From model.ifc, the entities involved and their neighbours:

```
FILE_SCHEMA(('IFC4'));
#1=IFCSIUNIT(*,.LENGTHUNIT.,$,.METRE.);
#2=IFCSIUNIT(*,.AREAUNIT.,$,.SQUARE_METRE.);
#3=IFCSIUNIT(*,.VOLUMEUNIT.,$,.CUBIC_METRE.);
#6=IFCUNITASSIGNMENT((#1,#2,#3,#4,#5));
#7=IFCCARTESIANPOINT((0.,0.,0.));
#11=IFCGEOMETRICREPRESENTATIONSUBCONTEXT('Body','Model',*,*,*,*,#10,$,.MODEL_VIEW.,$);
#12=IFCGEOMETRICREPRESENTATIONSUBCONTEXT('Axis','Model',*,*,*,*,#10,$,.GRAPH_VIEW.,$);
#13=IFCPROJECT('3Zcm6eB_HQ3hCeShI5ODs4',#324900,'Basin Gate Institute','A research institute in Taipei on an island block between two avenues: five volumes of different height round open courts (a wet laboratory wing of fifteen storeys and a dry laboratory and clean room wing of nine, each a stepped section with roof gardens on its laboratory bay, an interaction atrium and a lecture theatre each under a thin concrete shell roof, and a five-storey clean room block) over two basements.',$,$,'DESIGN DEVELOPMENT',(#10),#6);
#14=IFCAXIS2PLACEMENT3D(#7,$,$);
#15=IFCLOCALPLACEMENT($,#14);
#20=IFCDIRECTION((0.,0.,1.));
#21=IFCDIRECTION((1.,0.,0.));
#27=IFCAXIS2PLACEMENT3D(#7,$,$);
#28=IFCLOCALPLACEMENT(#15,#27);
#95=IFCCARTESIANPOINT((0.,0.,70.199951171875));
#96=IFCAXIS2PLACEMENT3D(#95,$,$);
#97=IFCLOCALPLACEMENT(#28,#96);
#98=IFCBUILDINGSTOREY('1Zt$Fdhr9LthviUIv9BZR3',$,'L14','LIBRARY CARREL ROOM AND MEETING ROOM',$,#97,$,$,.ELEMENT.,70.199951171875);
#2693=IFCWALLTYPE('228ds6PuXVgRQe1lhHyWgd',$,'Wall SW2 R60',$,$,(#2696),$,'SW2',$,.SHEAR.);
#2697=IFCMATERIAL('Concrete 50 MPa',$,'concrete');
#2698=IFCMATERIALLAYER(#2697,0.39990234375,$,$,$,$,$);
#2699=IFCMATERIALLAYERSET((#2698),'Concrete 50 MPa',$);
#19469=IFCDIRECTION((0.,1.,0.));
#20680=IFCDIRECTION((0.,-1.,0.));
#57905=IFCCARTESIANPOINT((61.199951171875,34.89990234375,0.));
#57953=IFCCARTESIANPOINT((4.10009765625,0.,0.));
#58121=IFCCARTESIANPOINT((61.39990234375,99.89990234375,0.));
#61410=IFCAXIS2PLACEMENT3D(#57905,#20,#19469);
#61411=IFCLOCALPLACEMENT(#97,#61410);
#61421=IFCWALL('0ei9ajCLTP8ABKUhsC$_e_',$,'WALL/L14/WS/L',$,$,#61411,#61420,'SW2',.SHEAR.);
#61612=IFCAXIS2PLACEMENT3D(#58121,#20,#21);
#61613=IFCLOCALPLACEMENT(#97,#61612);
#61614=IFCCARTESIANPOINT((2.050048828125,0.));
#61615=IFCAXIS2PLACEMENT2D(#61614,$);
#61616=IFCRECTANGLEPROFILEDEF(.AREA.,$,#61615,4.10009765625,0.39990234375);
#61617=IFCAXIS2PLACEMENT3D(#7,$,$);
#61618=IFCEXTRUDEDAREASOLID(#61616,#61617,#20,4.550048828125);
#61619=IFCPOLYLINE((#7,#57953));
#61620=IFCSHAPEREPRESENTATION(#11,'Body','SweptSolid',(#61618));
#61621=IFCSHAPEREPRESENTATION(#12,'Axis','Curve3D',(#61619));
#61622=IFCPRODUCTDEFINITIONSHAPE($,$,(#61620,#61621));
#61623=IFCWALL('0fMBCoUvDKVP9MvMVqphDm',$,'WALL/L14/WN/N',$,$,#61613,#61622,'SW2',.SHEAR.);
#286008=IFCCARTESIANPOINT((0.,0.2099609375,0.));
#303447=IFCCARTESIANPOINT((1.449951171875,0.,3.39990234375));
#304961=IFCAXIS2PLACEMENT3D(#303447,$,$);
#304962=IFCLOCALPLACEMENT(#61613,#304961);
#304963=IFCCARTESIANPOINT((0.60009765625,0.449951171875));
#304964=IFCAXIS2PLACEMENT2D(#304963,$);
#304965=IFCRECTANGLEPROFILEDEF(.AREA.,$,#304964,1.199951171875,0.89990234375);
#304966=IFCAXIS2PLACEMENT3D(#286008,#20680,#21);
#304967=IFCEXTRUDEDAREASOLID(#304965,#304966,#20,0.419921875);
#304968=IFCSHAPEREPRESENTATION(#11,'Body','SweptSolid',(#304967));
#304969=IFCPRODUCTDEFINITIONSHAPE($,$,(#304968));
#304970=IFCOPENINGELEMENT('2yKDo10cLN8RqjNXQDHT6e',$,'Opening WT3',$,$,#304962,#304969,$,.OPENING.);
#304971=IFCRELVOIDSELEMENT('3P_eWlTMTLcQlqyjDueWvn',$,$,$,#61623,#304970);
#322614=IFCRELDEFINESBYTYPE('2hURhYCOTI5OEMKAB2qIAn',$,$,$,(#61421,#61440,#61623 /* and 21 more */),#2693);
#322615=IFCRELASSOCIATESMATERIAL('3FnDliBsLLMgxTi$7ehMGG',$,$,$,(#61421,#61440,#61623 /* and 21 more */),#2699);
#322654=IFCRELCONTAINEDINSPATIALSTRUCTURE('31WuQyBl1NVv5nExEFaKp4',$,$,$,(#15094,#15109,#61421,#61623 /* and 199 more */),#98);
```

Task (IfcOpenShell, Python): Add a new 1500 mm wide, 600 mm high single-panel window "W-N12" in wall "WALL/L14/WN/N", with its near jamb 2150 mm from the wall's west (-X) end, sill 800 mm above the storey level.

```python
import numpy as np
import ifcopenshell
import ifcopenshell.api.feature
import ifcopenshell.api.geometry
import ifcopenshell.api.root
import ifcopenshell.api.spatial
import ifcopenshell.geom
import ifcopenshell.util.element
import ifcopenshell.util.placement
import ifcopenshell.util.representation
import ifcopenshell.util.shape
import ifcopenshell.util.unit

model = ifcopenshell.open("model.ifc")
unit_scale = ifcopenshell.util.unit.calculate_unit_scale(model)
settings = ifcopenshell.geom.settings()


def volume(element):
    """Net volume in cubic metres, openings subtracted."""
    shape = ifcopenshell.geom.create_shape(settings, element)
    return ifcopenshell.util.shape.get_volume(shape.geometry)


wall = model.by_guid("0fMBCoUvDKVP9MvMVqphDm")
storey = ifcopenshell.util.element.get_container(wall, ifc_class="IfcBuildingStorey")
context = ifcopenshell.util.representation.get_context(model, "Model", "Body", "MODEL_VIEW")
before = volume(wall)

width, height, from_end, sill = 1.5, 0.6, 2.15, 0.8  # metres

# The wall runs along its own X axis, and the end named is its -X end.
wall_shape = ifcopenshell.geom.create_shape(settings, wall)
x, y, z = ifcopenshell.util.shape.get_vertices(wall_shape.geometry).T
start = x.min() + from_end
face, thickness = float(y.min()), float(y.max() - y.min())
wall_matrix = ifcopenshell.util.placement.get_local_placement(wall.ObjectPlacement)
level = ifcopenshell.util.placement.get_local_placement(storey.ObjectPlacement)[2, 3]


def in_wall(x, y):
    """Placement at x, y metres in the wall's axes, at sill height."""
    matrix = wall_matrix.copy()
    matrix[:, 3] = wall_matrix @ np.array([x / unit_scale, y / unit_scale, 0.0, 1.0])
    matrix[2, 3] = level + sill / unit_scale
    return matrix


# Opening: a box that overshoots both wall faces by 50 mm.
opening = ifcopenshell.api.root.create_entity(model, ifc_class="IfcOpeningElement", predefined_type="OPENING")
box = ifcopenshell.api.geometry.add_wall_representation(
    model, context=context, length=width, height=height, thickness=thickness + 0.1
)
ifcopenshell.api.geometry.assign_representation(model, product=opening, representation=box)
ifcopenshell.api.geometry.edit_object_placement(model, product=opening, matrix=in_wall(start, face - 0.05), is_si=False)
ifcopenshell.api.feature.add_feature(model, feature=opening, element=wall)

window = ifcopenshell.api.root.create_entity(model, ifc_class="IfcWindow", name="W-N12", predefined_type="WINDOW")
window.OverallWidth, window.OverallHeight = width / unit_scale, height / unit_scale
window.PartitioningType = "SINGLE_PANEL"
body = ifcopenshell.api.geometry.add_window_representation(
    model,
    context=context,
    overall_width=window.OverallWidth,
    overall_height=window.OverallHeight,
    partition_type="SINGLE_PANEL",
)
ifcopenshell.api.geometry.assign_representation(model, product=window, representation=body)
ifcopenshell.api.spatial.assign_container(model, products=[window], relating_structure=storey)
ifcopenshell.api.feature.add_filling(model, opening=opening, element=window)

# Centre the window in the wall's thickness.
ifcopenshell.api.geometry.edit_object_placement(model, product=window, matrix=in_wall(start, face), is_si=False)
window_shape = ifcopenshell.geom.create_shape(settings, window)
depth = ifcopenshell.util.shape.get_vertices(window_shape.geometry)[:, 1]
offset = face + thickness / 2 - (depth.min() + depth.max()) / 2
ifcopenshell.api.geometry.edit_object_placement(model, product=window, matrix=in_wall(start, offset), is_si=False)

after = volume(wall)

print(f"wall volume {before:.3f} -> {after:.3f} m3")

model.write("model_edited.ifc")
```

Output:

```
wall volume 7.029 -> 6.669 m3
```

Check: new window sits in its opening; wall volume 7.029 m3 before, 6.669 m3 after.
